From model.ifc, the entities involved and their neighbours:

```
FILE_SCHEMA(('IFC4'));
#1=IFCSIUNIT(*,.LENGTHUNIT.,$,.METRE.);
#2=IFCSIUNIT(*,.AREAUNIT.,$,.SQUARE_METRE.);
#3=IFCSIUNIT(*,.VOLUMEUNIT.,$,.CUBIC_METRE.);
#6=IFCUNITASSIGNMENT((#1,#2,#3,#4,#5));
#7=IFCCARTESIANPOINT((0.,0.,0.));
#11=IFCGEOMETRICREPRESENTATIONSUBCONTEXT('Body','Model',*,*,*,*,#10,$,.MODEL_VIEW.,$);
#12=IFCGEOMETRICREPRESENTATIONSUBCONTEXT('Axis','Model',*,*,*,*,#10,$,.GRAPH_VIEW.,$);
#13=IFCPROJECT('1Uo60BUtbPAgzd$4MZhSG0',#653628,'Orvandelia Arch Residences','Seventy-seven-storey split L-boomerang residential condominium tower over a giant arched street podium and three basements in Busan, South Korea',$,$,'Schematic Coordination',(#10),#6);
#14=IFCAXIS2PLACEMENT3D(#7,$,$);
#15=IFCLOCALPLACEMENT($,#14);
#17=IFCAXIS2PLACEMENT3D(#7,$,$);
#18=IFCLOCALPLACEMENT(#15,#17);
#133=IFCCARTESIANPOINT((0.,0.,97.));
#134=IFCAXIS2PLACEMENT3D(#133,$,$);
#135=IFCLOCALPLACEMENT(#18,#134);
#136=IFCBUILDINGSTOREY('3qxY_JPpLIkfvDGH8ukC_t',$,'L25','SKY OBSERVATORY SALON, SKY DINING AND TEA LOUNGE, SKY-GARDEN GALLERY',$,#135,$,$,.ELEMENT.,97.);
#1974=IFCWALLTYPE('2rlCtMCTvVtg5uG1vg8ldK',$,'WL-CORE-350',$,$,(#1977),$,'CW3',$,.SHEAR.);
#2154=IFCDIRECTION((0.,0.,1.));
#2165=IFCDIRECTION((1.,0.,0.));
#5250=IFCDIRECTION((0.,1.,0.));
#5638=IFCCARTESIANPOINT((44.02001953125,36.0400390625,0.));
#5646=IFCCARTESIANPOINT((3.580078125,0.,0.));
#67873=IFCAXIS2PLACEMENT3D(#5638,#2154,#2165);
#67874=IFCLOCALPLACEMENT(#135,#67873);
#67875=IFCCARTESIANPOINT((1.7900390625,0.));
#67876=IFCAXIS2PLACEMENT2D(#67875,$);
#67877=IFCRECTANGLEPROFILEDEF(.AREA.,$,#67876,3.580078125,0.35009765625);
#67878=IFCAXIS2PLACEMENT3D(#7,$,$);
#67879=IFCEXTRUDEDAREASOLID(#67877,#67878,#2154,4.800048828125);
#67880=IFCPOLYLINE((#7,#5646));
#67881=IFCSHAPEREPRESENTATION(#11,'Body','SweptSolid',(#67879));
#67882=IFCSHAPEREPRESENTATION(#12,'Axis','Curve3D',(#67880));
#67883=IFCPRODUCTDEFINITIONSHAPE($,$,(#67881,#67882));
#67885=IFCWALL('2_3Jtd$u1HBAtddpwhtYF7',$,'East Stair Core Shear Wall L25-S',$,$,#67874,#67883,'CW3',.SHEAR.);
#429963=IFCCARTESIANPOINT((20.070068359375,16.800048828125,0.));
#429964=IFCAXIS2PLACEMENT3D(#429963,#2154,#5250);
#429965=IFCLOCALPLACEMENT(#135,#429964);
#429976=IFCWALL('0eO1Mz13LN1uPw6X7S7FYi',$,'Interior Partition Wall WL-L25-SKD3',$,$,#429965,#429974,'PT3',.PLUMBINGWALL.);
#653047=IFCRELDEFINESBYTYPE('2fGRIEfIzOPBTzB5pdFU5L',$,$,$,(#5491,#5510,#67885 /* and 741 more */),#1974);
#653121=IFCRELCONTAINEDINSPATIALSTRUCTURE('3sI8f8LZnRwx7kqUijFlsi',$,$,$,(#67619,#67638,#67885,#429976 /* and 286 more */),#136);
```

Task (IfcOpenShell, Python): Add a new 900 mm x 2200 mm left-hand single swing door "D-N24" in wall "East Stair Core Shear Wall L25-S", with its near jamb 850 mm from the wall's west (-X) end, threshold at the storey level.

```python
import numpy as np
import ifcopenshell
import ifcopenshell.api.feature
import ifcopenshell.api.geometry
import ifcopenshell.api.root
import ifcopenshell.api.spatial
import ifcopenshell.geom
import ifcopenshell.util.element
import ifcopenshell.util.placement
import ifcopenshell.util.representation
import ifcopenshell.util.shape
import ifcopenshell.util.unit

model = ifcopenshell.open("model.ifc")
unit_scale = ifcopenshell.util.unit.calculate_unit_scale(model)
settings = ifcopenshell.geom.settings()


def volume(element):
    """Net volume in cubic metres, openings subtracted."""
    shape = ifcopenshell.geom.create_shape(settings, element)
    return ifcopenshell.util.shape.get_volume(shape.geometry)


wall = model.by_guid("2_3Jtd$u1HBAtddpwhtYF7")
storey = ifcopenshell.util.element.get_container(wall, ifc_class="IfcBuildingStorey")
context = ifcopenshell.util.representation.get_context(model, "Model", "Body", "MODEL_VIEW")
before = volume(wall)

width, height, from_end, sill = 0.9, 2.2, 0.85, 0.0  # metres

# The wall runs along its own X axis, and the end named is its -X end.
wall_shape = ifcopenshell.geom.create_shape(settings, wall)
x, y, z = ifcopenshell.util.shape.get_vertices(wall_shape.geometry).T
start = x.min() + from_end
face, thickness = float(y.min()), float(y.max() - y.min())
wall_matrix = ifcopenshell.util.placement.get_local_placement(wall.ObjectPlacement)
level = ifcopenshell.util.placement.get_local_placement(storey.ObjectPlacement)[2, 3]


def in_wall(x, y):
    """Placement at x, y metres in the wall's axes, at sill height."""
    matrix = wall_matrix.copy()
    matrix[:, 3] = wall_matrix @ np.array([x / unit_scale, y / unit_scale, 0.0, 1.0])
    matrix[2, 3] = level + sill / unit_scale
    return matrix


# Opening: a box that overshoots both wall faces by 50 mm.
opening = ifcopenshell.api.root.create_entity(model, ifc_class="IfcOpeningElement", predefined_type="OPENING")
box = ifcopenshell.api.geometry.add_wall_representation(
    model, context=context, length=width, height=height, thickness=thickness + 0.1
)
ifcopenshell.api.geometry.assign_representation(model, product=opening, representation=box)
ifcopenshell.api.geometry.edit_object_placement(model, product=opening, matrix=in_wall(start, face - 0.05), is_si=False)
ifcopenshell.api.feature.add_feature(model, feature=opening, element=wall)

door = ifcopenshell.api.root.create_entity(model, ifc_class="IfcDoor", name="D-N24", predefined_type="DOOR")
door.OverallWidth, door.OverallHeight = width / unit_scale, height / unit_scale
door.OperationType = "SINGLE_SWING_LEFT"
body = ifcopenshell.api.geometry.add_door_representation(
    model,
    context=context,
    overall_width=door.OverallWidth,
    overall_height=door.OverallHeight,
    operation_type="SINGLE_SWING_LEFT",
    lining_properties={"LiningDepth": thickness / unit_scale, "ThresholdDepth": thickness / unit_scale},
)
ifcopenshell.api.geometry.assign_representation(model, product=door, representation=body)
ifcopenshell.api.spatial.assign_container(model, products=[door], relating_structure=storey)
ifcopenshell.api.feature.add_filling(model, opening=opening, element=door)

# The lining spans the wall, so the door starts at the wall face.
ifcopenshell.api.geometry.edit_object_placement(model, product=door, matrix=in_wall(start, face), is_si=False)

after = volume(wall)

print(f"wall volume {before:.3f} -> {after:.3f} m3")

model.write("model_v2.ifc")
```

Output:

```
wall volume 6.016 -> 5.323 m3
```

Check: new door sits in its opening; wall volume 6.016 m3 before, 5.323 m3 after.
